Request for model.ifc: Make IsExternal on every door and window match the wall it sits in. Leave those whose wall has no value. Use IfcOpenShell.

First a look at what the model holds.

```python
import ifcopenshell
import ifcopenshell.util.element

model = ifcopenshell.open("model.ifc")
print(model.schema)
seen = {}
for e in model.by_type("IfcDoor") + model.by_type("IfcWindow"):
    if not e.FillsVoids:
        continue
    host = e.FillsVoids[0].RelatingOpeningElement.VoidsElements[0].RelatingBuildingElement
    own = ifcopenshell.util.element.get_pset(e, f"Pset_{e.is_a()[3:].removesuffix('StandardCase')}Common", "IsExternal")
    wall = ifcopenshell.util.element.get_pset(host, "Pset_WallCommon", "IsExternal")
    seen[e.is_a(), own, wall] = seen.get((e.is_a(), own, wall), 0) + 1
for (cls, own, wall), count in sorted(seen.items(), key=str):
    print(count, cls, "IsExternal:", own, "| host wall:", wall)
```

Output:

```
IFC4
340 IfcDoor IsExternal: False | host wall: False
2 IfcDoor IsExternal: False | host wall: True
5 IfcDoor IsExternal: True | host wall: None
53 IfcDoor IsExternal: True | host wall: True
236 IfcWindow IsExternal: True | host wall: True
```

```python
import ifcopenshell
import ifcopenshell.api.pset
import ifcopenshell.util.element

model = ifcopenshell.open("model.ifc")

count = 0
for ifc_class, pset_name in (("IfcDoor", "Pset_DoorCommon"), ("IfcWindow", "Pset_WindowCommon")):
    for e in model.by_type(ifc_class):
        if not e.FillsVoids:
            continue
        host = e.FillsVoids[0].RelatingOpeningElement.VoidsElements[0].RelatingBuildingElement
        external = ifcopenshell.util.element.get_pset(host, "Pset_WallCommon", "IsExternal")
        if external is None or ifcopenshell.util.element.get_pset(e, pset_name, "IsExternal") == external:
            continue
        pset = ifcopenshell.api.pset.add_pset(model, product=e, name=pset_name)
        ifcopenshell.api.pset.edit_pset(model, pset=pset, properties={"IsExternal": external})
        count += 1

print(count, "updated")

model.write("model-out.ifc")
```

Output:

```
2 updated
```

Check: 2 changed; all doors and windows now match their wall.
